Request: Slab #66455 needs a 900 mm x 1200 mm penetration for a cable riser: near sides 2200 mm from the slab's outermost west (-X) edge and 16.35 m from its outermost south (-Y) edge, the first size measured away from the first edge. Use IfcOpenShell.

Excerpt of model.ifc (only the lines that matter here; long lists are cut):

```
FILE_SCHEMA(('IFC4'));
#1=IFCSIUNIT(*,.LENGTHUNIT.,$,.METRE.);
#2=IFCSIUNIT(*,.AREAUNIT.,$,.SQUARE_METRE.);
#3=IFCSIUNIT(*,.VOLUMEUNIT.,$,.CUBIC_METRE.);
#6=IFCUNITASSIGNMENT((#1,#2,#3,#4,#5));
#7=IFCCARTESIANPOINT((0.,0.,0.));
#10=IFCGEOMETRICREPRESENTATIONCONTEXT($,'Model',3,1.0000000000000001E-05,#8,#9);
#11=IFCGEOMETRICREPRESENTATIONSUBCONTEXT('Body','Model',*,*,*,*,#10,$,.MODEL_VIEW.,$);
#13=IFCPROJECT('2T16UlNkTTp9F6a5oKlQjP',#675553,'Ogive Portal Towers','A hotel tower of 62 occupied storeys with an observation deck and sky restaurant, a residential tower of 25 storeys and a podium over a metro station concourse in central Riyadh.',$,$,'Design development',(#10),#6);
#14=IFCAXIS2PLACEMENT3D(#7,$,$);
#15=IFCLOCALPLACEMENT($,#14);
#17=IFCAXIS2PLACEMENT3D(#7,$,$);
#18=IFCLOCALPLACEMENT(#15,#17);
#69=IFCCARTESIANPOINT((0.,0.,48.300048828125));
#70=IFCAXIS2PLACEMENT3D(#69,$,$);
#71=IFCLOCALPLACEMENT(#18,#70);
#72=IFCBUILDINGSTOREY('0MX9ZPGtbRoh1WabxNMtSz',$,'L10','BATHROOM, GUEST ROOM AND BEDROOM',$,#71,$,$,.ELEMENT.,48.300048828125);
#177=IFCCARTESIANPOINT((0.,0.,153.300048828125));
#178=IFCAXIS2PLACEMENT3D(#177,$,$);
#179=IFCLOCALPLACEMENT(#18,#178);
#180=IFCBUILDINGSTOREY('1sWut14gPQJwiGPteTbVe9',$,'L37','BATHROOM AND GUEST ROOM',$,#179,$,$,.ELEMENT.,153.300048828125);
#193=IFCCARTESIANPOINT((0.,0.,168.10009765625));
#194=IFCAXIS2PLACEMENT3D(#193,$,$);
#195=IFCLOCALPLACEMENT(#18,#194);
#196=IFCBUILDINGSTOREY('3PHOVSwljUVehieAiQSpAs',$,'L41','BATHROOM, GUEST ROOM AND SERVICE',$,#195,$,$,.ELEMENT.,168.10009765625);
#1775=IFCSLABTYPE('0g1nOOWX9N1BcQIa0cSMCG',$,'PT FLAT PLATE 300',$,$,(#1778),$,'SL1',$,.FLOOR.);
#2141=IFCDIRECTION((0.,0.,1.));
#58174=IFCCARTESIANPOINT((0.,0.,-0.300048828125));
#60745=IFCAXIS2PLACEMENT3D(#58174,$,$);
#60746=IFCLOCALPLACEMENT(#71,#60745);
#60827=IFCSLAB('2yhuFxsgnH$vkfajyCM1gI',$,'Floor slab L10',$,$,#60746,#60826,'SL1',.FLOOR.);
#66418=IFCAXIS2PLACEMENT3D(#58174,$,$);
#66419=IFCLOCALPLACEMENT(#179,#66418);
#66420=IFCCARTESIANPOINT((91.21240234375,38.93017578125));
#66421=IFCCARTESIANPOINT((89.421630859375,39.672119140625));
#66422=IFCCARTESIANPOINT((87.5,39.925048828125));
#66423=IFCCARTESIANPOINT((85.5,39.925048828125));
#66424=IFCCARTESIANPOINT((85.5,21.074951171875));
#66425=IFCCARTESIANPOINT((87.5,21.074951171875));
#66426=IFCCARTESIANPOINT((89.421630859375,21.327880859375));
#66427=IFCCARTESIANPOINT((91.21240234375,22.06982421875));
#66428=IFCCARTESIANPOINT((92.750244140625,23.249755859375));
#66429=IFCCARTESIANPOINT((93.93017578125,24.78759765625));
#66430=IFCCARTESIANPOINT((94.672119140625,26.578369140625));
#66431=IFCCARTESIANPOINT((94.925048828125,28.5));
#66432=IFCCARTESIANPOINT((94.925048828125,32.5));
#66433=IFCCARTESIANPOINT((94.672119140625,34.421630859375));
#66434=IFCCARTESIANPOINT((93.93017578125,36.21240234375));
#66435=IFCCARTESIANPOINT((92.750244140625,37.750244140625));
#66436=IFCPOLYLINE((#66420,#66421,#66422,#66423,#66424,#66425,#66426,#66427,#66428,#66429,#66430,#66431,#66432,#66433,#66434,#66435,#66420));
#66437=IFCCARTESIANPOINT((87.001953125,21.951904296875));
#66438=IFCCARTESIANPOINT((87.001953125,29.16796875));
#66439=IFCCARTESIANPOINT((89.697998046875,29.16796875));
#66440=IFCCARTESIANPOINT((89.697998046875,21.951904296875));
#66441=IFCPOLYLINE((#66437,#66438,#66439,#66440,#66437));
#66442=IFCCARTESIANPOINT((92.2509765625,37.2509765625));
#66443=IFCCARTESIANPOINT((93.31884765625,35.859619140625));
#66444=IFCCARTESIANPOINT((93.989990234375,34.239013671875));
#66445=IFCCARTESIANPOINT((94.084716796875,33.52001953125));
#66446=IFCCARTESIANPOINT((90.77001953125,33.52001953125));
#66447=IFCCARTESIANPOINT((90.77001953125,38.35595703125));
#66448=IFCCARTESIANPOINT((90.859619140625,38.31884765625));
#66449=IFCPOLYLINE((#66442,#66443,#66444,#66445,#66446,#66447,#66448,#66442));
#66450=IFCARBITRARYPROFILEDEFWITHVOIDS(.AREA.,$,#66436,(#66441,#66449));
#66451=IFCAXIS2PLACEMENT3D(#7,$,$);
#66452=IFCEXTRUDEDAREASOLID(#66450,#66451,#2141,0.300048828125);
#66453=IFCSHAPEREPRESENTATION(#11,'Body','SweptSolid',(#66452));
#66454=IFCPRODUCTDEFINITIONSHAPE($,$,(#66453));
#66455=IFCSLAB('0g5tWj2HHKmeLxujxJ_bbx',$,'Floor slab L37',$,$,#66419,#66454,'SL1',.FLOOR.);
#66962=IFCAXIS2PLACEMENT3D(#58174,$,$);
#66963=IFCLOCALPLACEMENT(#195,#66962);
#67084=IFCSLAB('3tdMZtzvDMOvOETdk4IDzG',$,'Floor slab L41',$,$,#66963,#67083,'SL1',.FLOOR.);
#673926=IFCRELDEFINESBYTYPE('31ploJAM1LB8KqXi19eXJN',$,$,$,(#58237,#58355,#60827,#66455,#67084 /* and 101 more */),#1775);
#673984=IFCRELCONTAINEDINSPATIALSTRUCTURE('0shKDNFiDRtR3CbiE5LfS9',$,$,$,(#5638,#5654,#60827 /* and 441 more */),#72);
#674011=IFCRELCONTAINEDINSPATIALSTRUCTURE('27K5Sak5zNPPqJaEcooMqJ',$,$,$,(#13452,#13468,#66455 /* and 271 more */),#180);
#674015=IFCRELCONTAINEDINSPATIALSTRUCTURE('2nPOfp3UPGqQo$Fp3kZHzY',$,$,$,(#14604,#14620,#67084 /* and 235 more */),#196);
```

```python
import numpy as np
import ifcopenshell
import ifcopenshell.api.feature
import ifcopenshell.api.geometry
import ifcopenshell.api.root
import ifcopenshell.geom
import ifcopenshell.util.placement
import ifcopenshell.util.representation
import ifcopenshell.util.shape
import ifcopenshell.util.unit

model = ifcopenshell.open("model.ifc")
unit_scale = ifcopenshell.util.unit.calculate_unit_scale(model)
settings = ifcopenshell.geom.settings()


def volume(element):
    """Net volume in cubic metres, openings subtracted."""
    shape = ifcopenshell.geom.create_shape(settings, element)
    return ifcopenshell.util.shape.get_volume(shape.geometry)


slab = model.by_guid("0g5tWj2HHKmeLxujxJ_bbx")
before = volume(slab)

# Extent in the slab's own axes, in metres. The edges named are its -X and -Y sides.
slab_shape = ifcopenshell.geom.create_shape(settings, slab)
vertices = ifcopenshell.util.shape.get_vertices(slab_shape.geometry)
x_min, y_min, bottom = vertices.min(axis=0)
top = vertices[:, 2].max()

opening = ifcopenshell.api.root.create_entity(model, ifc_class="IfcOpeningElement", name="Cable riser opening", predefined_type="OPENING")
context = ifcopenshell.util.representation.get_context(model, "Model", "Body", "MODEL_VIEW")
width, depth = 0.9, 1.2
outline = [(0.0, 0.0), (width, 0.0), (width, depth), (0.0, depth), (0.0, 0.0)]
# Overshoot both faces by 50 mm so the cut is clean.
shape = ifcopenshell.api.geometry.add_slab_representation(
    model, context=context, depth=top - bottom + 0.1, polyline=outline
)
ifcopenshell.api.geometry.assign_representation(model, product=opening, representation=shape)

matrix = ifcopenshell.util.placement.get_local_placement(slab.ObjectPlacement)
matrix[:, 3] = matrix @ np.append(np.array([x_min + 2.2, y_min + 16.35, bottom - 0.05]) / unit_scale, 1.0)
ifcopenshell.api.geometry.edit_object_placement(model, product=opening, matrix=matrix, is_si=False)
ifcopenshell.api.feature.add_feature(model, feature=opening, element=slab)

after = volume(slab)

print(f"slab volume {before:.3f} -> {after:.3f} m3")

model.write("model_v2.ifc")
```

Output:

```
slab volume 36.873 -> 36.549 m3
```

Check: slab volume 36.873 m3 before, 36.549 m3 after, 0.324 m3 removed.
